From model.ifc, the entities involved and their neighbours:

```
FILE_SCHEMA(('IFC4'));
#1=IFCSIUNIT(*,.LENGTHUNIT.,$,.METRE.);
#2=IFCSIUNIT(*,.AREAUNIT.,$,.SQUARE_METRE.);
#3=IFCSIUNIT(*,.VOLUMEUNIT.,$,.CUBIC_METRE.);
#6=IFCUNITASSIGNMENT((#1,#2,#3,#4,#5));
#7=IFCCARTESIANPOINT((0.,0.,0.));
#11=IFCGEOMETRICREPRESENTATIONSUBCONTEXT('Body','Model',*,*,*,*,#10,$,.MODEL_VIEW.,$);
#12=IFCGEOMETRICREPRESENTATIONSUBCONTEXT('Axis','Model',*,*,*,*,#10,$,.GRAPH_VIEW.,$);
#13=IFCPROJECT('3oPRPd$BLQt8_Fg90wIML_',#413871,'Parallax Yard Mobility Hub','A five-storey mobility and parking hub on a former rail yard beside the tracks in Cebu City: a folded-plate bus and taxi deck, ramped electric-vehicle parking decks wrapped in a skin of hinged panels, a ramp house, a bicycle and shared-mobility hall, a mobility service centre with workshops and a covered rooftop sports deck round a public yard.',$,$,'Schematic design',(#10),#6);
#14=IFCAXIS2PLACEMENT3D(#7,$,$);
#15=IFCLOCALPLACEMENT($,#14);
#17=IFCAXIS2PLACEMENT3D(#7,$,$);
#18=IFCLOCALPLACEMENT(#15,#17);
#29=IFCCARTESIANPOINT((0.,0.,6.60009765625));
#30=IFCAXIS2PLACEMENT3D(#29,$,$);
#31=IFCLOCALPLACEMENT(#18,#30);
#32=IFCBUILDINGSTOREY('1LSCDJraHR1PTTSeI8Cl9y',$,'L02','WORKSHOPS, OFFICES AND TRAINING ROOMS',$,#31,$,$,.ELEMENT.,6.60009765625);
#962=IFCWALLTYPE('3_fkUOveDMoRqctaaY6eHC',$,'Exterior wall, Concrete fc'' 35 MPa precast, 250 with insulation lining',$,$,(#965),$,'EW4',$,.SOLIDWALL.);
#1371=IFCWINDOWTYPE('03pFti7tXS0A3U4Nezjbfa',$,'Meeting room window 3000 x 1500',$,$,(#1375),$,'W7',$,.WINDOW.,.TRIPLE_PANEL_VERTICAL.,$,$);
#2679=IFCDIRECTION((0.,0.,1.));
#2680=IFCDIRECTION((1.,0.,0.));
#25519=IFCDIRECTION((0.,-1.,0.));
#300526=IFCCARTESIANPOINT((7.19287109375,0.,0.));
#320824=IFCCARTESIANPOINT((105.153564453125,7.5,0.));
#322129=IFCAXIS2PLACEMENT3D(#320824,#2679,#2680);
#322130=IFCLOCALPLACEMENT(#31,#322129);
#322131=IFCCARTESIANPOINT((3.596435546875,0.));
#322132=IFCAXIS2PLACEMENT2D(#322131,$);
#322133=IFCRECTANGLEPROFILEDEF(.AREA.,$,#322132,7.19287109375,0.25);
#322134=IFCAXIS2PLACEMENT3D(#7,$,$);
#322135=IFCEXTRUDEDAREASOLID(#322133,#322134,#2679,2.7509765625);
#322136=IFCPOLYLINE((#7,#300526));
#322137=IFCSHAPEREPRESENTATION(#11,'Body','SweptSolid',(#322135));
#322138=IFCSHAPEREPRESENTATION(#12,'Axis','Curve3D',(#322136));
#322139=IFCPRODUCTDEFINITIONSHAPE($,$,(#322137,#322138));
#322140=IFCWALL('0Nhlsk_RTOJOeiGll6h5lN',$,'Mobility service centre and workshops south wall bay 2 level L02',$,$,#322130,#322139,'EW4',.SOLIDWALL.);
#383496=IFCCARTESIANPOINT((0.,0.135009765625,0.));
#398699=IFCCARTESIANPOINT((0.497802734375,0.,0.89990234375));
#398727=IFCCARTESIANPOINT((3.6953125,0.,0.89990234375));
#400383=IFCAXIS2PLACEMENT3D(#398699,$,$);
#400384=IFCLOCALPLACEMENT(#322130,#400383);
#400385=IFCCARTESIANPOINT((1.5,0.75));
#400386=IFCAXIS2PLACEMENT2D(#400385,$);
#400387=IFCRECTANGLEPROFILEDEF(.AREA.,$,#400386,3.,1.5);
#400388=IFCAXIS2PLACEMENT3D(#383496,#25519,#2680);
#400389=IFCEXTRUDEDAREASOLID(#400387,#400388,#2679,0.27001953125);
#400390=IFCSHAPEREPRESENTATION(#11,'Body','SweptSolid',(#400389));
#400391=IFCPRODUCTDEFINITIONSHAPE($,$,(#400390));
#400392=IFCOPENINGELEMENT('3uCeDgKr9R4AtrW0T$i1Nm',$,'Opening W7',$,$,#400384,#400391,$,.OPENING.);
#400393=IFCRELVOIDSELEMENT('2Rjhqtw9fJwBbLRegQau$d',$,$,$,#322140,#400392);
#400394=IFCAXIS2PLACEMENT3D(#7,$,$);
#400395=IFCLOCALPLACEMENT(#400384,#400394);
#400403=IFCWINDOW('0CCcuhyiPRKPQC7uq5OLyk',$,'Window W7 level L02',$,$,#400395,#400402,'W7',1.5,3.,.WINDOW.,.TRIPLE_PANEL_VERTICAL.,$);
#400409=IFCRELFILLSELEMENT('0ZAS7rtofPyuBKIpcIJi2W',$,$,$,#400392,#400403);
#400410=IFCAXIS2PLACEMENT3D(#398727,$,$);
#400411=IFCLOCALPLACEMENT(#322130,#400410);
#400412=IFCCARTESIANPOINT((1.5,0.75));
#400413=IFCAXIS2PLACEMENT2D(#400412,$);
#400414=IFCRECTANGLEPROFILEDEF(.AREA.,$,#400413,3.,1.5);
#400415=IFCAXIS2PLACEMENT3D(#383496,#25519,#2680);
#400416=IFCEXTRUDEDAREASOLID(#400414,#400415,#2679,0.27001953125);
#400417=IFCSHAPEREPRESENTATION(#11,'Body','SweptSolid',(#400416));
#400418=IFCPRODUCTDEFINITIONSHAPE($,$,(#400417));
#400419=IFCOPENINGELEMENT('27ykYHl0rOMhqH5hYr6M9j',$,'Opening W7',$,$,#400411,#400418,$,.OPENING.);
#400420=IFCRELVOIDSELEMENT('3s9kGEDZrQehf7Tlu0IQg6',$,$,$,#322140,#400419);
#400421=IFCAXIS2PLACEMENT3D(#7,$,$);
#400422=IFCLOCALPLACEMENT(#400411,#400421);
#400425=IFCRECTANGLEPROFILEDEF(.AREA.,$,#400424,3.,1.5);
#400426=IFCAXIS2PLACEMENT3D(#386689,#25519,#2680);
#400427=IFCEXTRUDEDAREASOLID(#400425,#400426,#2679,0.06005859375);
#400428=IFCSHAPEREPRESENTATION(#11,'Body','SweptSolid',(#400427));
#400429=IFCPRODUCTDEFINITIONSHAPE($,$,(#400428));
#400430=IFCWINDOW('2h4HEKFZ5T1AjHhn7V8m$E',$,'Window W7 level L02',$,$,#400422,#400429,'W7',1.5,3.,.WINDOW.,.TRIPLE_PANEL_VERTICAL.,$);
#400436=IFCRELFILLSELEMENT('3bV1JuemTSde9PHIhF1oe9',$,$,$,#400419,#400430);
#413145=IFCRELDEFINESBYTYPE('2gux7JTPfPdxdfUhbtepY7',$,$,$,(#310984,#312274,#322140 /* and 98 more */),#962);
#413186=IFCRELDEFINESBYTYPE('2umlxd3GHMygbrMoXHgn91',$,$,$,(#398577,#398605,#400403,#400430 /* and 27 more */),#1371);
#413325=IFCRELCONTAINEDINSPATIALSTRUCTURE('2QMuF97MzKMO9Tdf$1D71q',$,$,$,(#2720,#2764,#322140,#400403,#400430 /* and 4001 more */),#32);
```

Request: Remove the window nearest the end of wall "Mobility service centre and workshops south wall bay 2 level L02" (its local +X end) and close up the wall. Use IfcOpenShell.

```python
import ifcopenshell
import ifcopenshell.api.feature
import ifcopenshell.api.root
import ifcopenshell.geom
import ifcopenshell.util.shape

model = ifcopenshell.open("model.ifc")
settings = ifcopenshell.geom.settings()


def volume(element):
    """Net volume in cubic metres, openings subtracted."""
    shape = ifcopenshell.geom.create_shape(settings, element)
    return ifcopenshell.util.shape.get_volume(shape.geometry)


window = model.by_guid("2h4HEKFZ5T1AjHhn7V8m$E")
opening = window.FillsVoids[0].RelatingOpeningElement
wall = opening.VoidsElements[0].RelatingBuildingElement
before = volume(wall)

ifcopenshell.api.root.remove_product(model, product=window)
ifcopenshell.api.feature.remove_feature(model, feature=opening)

after = volume(wall)

print(f"wall volume {before:.3f} -> {after:.3f} m3")

model.write("model-out.ifc")
```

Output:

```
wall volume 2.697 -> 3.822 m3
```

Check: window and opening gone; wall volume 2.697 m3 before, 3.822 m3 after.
